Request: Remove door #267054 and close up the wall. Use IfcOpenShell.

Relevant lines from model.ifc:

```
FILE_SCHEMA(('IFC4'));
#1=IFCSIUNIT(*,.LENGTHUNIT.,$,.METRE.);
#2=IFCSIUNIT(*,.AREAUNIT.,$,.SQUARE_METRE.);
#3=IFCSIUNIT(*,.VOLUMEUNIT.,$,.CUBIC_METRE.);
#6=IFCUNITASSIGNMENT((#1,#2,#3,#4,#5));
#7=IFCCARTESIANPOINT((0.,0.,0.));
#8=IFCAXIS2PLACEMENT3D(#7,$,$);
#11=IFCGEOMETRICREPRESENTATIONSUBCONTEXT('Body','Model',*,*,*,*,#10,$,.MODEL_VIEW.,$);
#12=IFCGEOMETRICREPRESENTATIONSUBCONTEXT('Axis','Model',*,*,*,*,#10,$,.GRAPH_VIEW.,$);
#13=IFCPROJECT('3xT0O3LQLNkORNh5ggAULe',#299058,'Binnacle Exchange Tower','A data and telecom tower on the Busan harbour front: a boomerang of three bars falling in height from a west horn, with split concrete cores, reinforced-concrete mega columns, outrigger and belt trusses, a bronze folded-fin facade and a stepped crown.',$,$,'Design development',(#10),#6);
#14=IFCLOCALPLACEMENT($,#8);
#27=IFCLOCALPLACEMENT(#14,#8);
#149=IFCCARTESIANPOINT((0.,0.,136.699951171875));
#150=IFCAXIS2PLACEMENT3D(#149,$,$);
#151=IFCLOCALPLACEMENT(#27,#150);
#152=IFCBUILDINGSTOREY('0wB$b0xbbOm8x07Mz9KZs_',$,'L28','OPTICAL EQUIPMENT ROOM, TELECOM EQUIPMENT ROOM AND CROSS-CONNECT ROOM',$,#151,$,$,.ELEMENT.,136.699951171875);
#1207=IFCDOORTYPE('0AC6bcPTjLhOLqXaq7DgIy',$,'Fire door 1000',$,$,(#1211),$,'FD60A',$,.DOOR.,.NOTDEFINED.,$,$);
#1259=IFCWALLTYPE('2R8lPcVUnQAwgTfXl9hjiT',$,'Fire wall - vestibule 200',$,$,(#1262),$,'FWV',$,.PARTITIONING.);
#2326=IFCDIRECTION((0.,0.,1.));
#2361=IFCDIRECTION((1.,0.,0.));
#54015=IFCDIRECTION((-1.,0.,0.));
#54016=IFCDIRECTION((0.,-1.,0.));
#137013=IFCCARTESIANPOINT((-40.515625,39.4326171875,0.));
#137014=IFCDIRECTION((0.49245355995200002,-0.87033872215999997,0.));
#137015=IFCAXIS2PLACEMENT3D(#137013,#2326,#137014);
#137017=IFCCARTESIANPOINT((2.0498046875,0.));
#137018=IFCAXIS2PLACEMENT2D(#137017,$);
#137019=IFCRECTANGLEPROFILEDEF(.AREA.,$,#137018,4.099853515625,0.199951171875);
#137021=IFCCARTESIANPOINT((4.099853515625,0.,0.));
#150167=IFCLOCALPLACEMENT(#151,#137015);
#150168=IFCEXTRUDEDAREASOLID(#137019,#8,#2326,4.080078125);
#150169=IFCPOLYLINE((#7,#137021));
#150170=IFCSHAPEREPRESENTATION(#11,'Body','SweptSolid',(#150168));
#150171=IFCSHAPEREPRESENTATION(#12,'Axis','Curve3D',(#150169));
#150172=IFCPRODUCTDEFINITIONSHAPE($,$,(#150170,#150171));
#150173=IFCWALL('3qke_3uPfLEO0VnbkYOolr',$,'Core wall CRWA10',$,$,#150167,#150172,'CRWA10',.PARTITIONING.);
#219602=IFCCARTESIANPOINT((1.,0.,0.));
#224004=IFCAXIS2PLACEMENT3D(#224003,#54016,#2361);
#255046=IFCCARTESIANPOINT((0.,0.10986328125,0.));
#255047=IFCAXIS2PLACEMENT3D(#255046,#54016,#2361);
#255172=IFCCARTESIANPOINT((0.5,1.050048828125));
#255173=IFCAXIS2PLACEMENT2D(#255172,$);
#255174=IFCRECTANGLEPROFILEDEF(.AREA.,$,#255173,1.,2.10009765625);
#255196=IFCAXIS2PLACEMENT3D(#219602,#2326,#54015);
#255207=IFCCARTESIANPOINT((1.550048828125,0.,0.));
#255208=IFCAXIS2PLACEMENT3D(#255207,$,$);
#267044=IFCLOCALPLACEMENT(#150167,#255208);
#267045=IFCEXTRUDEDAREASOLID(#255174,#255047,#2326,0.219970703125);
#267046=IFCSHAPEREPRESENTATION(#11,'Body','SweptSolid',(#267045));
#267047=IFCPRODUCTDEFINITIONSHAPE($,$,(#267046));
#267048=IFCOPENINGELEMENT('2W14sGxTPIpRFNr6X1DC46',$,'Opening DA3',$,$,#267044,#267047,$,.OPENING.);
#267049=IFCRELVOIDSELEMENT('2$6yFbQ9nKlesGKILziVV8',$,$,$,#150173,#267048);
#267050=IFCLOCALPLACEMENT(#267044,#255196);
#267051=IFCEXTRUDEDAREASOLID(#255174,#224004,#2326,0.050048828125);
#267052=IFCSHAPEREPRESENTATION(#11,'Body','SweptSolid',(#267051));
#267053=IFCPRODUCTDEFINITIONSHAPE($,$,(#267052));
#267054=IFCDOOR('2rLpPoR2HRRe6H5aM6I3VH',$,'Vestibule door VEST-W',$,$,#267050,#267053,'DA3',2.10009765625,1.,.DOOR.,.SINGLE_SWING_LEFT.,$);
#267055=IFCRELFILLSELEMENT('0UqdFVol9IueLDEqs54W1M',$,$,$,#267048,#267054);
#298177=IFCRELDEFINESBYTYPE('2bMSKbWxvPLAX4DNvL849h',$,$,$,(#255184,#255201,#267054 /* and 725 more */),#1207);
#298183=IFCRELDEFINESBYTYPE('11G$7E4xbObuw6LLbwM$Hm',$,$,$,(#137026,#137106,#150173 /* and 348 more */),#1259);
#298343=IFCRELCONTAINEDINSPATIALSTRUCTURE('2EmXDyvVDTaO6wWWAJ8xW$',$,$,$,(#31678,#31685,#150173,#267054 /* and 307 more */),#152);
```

```python
import ifcopenshell
import ifcopenshell.api.feature
import ifcopenshell.api.root
import ifcopenshell.geom
import ifcopenshell.util.shape

model = ifcopenshell.open("model.ifc")
settings = ifcopenshell.geom.settings()


def volume(element):
    """Net volume in cubic metres, openings subtracted."""
    shape = ifcopenshell.geom.create_shape(settings, element)
    return ifcopenshell.util.shape.get_volume(shape.geometry)


door = model.by_guid("2rLpPoR2HRRe6H5aM6I3VH")
opening = door.FillsVoids[0].RelatingOpeningElement
wall = opening.VoidsElements[0].RelatingBuildingElement
before = volume(wall)

ifcopenshell.api.root.remove_product(model, product=door)
ifcopenshell.api.feature.remove_feature(model, feature=opening)

after = volume(wall)

print(f"wall volume {before:.3f} -> {after:.3f} m3")

model.write("model-out.ifc")
```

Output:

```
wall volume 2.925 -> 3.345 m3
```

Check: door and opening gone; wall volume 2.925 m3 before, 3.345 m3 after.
